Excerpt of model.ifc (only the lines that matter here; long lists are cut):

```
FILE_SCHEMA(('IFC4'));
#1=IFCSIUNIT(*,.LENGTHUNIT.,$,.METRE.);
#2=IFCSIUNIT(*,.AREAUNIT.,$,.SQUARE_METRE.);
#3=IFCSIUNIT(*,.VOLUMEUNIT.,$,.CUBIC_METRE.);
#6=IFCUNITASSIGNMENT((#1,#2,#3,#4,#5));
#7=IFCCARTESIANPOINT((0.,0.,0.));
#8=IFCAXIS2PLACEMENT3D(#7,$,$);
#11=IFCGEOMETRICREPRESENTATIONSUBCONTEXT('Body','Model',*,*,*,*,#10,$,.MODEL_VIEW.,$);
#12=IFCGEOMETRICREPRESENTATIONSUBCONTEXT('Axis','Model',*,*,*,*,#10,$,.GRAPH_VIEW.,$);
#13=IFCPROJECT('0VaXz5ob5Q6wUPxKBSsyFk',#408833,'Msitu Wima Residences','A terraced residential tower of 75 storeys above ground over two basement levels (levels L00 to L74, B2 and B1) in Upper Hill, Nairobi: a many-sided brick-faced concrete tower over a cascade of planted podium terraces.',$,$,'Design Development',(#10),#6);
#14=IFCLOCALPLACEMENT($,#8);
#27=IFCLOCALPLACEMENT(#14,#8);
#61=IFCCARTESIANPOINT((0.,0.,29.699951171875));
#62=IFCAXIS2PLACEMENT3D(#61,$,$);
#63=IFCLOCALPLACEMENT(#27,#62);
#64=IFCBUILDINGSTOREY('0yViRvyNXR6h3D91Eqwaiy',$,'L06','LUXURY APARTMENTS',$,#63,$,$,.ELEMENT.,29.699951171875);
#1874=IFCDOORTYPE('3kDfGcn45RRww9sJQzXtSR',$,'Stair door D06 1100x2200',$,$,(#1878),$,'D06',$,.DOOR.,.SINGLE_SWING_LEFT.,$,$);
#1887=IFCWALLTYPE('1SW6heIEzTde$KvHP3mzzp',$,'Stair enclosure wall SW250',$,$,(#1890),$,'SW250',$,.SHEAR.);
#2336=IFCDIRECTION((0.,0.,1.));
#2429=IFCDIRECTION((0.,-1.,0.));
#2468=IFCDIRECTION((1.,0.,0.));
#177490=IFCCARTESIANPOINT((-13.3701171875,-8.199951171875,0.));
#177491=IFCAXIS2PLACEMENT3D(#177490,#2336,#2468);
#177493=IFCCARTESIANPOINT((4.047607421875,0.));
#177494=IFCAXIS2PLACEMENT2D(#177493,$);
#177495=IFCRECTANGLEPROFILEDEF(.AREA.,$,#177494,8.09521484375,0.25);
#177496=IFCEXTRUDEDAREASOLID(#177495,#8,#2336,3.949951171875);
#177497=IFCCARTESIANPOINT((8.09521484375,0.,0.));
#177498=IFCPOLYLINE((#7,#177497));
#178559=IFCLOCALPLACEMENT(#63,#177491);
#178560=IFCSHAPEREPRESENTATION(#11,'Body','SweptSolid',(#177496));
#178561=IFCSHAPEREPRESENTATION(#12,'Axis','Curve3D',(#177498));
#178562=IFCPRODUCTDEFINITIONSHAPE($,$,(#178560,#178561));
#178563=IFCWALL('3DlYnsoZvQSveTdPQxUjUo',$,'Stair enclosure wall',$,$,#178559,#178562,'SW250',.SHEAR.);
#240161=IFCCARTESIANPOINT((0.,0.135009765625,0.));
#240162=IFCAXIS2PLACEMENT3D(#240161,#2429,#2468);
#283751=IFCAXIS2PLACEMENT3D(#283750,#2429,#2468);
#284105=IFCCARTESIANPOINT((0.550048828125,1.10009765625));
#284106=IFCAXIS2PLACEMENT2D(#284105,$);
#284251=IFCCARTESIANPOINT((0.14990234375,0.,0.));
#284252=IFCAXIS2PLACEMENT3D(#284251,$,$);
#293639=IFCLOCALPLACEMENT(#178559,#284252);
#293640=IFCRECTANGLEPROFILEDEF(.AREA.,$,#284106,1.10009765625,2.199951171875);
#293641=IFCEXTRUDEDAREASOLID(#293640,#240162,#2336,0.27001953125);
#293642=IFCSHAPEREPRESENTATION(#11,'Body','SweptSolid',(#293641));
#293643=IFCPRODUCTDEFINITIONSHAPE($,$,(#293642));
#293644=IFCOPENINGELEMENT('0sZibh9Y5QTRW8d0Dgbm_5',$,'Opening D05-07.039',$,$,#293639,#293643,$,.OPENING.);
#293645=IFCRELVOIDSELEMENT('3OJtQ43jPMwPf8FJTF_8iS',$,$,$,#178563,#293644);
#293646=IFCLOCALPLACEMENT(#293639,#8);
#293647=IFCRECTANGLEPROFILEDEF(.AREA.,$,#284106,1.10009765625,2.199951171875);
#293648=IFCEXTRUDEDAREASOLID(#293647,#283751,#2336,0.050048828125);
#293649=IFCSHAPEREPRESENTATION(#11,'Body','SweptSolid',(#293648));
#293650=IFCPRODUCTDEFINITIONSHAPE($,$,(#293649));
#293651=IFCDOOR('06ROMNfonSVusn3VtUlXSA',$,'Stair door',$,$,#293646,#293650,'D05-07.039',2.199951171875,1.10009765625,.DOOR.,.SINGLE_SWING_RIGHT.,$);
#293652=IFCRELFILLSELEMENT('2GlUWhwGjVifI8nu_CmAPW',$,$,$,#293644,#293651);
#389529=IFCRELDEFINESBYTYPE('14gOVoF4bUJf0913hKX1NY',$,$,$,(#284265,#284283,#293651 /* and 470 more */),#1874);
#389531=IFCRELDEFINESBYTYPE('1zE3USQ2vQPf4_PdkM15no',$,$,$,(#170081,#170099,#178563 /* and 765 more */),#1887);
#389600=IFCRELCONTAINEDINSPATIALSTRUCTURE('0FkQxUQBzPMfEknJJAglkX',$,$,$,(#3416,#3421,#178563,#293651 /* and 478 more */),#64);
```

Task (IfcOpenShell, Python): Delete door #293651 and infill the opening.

```python
import ifcopenshell
import ifcopenshell.api.feature
import ifcopenshell.api.root
import ifcopenshell.geom
import ifcopenshell.util.shape

model = ifcopenshell.open("model.ifc")
settings = ifcopenshell.geom.settings()


def volume(element):
    """Net volume in cubic metres, openings subtracted."""
    shape = ifcopenshell.geom.create_shape(settings, element)
    return ifcopenshell.util.shape.get_volume(shape.geometry)


door = model.by_id(293651)
opening = door.FillsVoids[0].RelatingOpeningElement
wall = opening.VoidsElements[0].RelatingBuildingElement
before = volume(wall)

ifcopenshell.api.root.remove_product(model, product=door)
ifcopenshell.api.feature.remove_feature(model, feature=opening)

after = volume(wall)

print(f"wall volume {before:.3f} -> {after:.3f} m3")

model.write("model_rev.ifc")
```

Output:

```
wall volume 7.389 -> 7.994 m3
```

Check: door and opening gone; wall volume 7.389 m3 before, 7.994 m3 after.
